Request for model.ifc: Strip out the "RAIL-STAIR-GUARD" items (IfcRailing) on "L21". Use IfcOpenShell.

First a look at what the model holds.

```python
import ifcopenshell
import ifcopenshell.util.element

model = ifcopenshell.open("model.ifc")
print(model.schema)
storey = next(s for s in model.by_type("IfcBuildingStorey") if s.Name == "L21")
railings = [e for e in ifcopenshell.util.element.get_decomposition(storey) if e.is_a("IfcRailing")]
seen = {}
for e in railings:
    element_type = ifcopenshell.util.element.get_type(e)
    name = element_type.Name if element_type not in (None, e) else None
    seen[name] = seen.get(name, 0) + 1
for name, count in sorted(seen.items(), key=str):
    print(count, "x", name)
```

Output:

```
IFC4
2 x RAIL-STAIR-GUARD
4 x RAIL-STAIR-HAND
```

```python
import ifcopenshell
import ifcopenshell.api.root
import ifcopenshell.util.element

model = ifcopenshell.open("model.ifc")

storey = next(s for s in model.by_type("IfcBuildingStorey") if s.Name == "L21")
railings = [e for e in ifcopenshell.util.element.get_decomposition(storey) if e.is_a("IfcRailing")]
targets = [e for e in railings if (t := ifcopenshell.util.element.get_type(e)) not in (None, e) and t.Name == "RAIL-STAIR-GUARD"]

for e in targets:
    ifcopenshell.api.root.remove_product(model, product=e)
print(len(targets), "removed")

model.write("model-out.ifc")
```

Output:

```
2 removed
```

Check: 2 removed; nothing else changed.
